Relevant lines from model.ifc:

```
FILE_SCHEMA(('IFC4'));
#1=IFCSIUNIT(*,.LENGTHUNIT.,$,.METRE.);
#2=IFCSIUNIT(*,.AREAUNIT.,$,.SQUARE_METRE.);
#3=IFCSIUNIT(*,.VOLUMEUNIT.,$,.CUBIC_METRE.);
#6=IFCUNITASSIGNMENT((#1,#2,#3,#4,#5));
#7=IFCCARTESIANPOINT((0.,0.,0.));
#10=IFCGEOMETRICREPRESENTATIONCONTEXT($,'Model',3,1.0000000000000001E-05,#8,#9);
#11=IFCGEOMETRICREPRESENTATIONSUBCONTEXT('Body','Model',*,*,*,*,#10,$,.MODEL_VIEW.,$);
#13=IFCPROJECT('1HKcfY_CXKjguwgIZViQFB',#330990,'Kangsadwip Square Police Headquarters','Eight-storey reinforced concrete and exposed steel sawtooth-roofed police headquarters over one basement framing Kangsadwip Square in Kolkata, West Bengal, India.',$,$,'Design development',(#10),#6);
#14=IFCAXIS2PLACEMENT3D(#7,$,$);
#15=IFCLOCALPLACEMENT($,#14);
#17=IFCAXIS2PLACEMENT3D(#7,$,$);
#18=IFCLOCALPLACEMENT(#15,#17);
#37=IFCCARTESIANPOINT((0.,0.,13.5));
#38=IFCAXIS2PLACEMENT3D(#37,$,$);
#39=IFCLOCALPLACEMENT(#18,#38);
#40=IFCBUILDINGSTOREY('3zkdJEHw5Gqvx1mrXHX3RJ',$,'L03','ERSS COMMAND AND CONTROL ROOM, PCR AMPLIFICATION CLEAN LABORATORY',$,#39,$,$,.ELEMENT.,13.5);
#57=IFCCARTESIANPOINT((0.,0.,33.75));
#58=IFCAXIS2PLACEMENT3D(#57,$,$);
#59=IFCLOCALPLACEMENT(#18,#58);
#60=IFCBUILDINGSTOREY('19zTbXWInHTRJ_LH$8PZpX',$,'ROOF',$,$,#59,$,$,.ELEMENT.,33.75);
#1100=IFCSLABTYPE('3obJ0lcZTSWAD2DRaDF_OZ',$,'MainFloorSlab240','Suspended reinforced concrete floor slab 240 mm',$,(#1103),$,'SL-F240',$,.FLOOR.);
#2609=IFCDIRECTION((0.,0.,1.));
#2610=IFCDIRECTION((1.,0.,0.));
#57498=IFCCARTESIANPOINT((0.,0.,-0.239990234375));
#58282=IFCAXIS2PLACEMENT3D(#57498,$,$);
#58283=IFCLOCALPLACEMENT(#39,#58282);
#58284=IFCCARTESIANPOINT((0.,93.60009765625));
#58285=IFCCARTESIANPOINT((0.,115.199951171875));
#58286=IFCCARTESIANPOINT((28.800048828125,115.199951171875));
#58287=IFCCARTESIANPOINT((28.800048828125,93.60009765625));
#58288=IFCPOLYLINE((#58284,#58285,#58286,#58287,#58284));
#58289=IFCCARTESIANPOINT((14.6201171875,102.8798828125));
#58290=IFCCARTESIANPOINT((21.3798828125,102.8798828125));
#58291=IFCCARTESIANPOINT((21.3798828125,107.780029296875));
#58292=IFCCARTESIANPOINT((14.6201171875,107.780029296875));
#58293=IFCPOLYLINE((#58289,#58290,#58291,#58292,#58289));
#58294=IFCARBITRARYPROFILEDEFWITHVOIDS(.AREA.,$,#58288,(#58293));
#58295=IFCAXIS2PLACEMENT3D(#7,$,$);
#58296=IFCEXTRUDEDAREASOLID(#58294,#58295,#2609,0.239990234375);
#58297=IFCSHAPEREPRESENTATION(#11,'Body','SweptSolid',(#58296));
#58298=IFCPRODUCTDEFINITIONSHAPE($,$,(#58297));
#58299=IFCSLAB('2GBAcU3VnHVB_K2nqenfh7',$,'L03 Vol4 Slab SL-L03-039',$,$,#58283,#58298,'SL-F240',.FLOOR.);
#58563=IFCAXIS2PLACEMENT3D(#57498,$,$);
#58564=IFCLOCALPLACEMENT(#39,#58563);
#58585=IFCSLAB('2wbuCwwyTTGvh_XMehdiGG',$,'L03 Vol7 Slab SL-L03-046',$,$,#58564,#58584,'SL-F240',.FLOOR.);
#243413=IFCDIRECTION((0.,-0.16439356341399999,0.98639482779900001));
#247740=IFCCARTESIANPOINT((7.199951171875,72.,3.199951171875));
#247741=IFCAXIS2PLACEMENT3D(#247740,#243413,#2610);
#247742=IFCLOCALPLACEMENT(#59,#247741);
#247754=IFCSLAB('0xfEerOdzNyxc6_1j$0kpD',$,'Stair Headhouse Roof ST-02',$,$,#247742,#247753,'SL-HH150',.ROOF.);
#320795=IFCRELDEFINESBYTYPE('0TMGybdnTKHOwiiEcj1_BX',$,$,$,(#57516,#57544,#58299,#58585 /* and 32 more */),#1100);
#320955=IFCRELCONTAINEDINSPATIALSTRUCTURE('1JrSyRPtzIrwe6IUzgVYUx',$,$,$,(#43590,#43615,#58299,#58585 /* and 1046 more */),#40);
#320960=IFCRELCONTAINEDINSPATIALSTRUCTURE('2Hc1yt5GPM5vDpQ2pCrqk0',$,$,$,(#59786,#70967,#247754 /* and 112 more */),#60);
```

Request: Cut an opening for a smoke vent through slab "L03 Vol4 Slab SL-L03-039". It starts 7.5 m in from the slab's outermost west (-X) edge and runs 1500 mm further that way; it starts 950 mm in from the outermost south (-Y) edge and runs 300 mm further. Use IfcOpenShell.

```python
import numpy as np
import ifcopenshell
import ifcopenshell.api.feature
import ifcopenshell.api.geometry
import ifcopenshell.api.root
import ifcopenshell.geom
import ifcopenshell.util.placement
import ifcopenshell.util.representation
import ifcopenshell.util.shape
import ifcopenshell.util.unit

model = ifcopenshell.open("model.ifc")
unit_scale = ifcopenshell.util.unit.calculate_unit_scale(model)
settings = ifcopenshell.geom.settings()


def volume(element):
    """Net volume in cubic metres, openings subtracted."""
    shape = ifcopenshell.geom.create_shape(settings, element)
    return ifcopenshell.util.shape.get_volume(shape.geometry)


slab = model.by_id(58299)
before = volume(slab)

# Extent in the slab's own axes, in metres. The edges named are its -X and -Y sides.
slab_shape = ifcopenshell.geom.create_shape(settings, slab)
vertices = ifcopenshell.util.shape.get_vertices(slab_shape.geometry)
x_min, y_min, bottom = vertices.min(axis=0)
top = vertices[:, 2].max()

opening = ifcopenshell.api.root.create_entity(model, ifc_class="IfcOpeningElement", name="Smoke vent opening", predefined_type="OPENING")
context = ifcopenshell.util.representation.get_context(model, "Model", "Body", "MODEL_VIEW")
width, depth = 1.5, 0.3
outline = [(0.0, 0.0), (width, 0.0), (width, depth), (0.0, depth), (0.0, 0.0)]
# Overshoot both faces by 50 mm so the cut is clean.
shape = ifcopenshell.api.geometry.add_slab_representation(
    model, context=context, depth=top - bottom + 0.1, polyline=outline
)
ifcopenshell.api.geometry.assign_representation(model, product=opening, representation=shape)

matrix = ifcopenshell.util.placement.get_local_placement(slab.ObjectPlacement)
matrix[:, 3] = matrix @ np.append(np.array([x_min + 7.5, y_min + 0.95, bottom - 0.05]) / unit_scale, 1.0)
ifcopenshell.api.geometry.edit_object_placement(model, product=opening, matrix=matrix, is_si=False)
ifcopenshell.api.feature.add_feature(model, feature=opening, element=slab)

after = volume(slab)

print(f"slab volume {before:.3f} -> {after:.3f} m3")

model.write("model_rev.ifc")
```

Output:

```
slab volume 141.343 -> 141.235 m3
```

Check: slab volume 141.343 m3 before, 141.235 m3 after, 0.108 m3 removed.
